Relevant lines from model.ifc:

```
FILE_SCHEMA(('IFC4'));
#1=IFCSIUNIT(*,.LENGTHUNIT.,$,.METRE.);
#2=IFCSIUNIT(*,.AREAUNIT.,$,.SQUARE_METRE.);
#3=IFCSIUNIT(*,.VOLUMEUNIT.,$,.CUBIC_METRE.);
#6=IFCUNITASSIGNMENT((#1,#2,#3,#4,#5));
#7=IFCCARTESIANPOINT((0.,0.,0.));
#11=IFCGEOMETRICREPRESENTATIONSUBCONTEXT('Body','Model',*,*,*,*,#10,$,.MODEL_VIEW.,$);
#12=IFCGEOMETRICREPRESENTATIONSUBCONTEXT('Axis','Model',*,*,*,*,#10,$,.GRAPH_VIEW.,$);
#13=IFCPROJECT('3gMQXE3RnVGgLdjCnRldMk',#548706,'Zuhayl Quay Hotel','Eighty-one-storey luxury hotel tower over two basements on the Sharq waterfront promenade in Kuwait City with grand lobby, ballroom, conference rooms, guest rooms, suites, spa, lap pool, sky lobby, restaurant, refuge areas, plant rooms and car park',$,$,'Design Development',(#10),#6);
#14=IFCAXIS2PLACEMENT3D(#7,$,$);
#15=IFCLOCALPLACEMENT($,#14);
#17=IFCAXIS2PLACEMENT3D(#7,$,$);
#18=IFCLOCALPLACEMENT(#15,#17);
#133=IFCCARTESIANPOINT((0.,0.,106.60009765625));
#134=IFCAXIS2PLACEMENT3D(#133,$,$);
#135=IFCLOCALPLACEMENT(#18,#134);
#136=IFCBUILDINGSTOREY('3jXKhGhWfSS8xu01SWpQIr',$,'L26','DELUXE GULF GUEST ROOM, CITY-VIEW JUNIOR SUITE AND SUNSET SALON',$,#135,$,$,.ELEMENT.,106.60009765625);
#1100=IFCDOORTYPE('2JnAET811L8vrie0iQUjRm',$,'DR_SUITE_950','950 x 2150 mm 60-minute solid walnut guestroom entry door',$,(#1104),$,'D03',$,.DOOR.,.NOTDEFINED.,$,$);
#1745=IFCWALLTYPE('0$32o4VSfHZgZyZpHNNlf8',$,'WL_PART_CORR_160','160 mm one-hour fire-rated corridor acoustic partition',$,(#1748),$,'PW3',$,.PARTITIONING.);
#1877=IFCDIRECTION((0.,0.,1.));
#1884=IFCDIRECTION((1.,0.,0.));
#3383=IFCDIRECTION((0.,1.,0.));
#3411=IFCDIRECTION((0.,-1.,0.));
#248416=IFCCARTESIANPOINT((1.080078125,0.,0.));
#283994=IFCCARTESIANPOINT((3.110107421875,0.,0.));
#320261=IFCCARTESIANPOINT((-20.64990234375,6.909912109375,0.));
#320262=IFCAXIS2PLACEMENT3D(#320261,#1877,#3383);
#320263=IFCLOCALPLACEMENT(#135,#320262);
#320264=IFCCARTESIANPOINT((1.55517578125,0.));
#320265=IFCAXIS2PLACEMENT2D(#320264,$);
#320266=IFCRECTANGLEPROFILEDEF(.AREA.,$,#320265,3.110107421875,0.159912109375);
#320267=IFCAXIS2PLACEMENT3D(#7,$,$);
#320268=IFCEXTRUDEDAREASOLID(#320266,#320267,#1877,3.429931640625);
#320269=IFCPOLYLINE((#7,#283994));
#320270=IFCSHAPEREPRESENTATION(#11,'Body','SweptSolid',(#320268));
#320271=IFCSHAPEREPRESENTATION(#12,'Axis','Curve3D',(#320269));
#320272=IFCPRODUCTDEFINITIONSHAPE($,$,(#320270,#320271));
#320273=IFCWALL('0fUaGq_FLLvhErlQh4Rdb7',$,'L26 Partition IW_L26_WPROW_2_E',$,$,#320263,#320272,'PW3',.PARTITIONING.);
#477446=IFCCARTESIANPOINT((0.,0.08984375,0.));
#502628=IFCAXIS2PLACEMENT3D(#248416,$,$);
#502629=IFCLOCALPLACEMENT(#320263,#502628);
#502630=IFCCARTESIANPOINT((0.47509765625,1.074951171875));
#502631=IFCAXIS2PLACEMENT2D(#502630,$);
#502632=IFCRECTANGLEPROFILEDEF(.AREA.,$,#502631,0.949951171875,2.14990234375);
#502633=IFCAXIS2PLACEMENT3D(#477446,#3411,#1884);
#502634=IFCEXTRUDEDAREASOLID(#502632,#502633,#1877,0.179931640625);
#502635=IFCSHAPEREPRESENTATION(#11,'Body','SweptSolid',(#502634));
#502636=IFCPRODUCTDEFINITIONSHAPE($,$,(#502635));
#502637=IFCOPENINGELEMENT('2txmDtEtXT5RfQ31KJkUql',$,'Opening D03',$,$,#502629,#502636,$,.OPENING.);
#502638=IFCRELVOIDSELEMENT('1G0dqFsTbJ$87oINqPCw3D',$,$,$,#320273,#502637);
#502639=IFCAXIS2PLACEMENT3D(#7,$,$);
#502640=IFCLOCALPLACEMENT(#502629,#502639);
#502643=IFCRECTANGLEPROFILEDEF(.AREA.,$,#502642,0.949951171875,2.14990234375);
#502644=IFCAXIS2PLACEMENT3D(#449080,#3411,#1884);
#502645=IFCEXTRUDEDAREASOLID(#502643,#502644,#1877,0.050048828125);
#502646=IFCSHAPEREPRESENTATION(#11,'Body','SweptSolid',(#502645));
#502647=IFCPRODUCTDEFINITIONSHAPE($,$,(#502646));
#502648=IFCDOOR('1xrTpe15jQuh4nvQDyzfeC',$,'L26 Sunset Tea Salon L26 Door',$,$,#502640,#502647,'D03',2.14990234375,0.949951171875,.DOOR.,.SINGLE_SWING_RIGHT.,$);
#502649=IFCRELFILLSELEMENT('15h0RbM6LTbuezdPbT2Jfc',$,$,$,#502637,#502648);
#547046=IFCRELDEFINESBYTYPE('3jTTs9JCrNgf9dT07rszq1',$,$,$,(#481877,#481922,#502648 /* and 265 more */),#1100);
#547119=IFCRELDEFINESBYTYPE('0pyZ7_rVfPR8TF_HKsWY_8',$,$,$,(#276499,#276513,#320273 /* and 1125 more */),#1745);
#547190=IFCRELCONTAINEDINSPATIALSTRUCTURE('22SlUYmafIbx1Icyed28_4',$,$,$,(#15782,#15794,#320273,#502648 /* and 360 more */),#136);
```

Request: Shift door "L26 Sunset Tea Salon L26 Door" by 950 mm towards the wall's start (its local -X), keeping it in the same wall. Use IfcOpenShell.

```python
import ifcopenshell
import ifcopenshell.api.geometry
import ifcopenshell.util.placement
import ifcopenshell.util.unit

model = ifcopenshell.open("model.ifc")
unit_scale = ifcopenshell.util.unit.calculate_unit_scale(model)

door = model.by_guid("1xrTpe15jQuh4nvQDyzfeC")
opening = door.FillsVoids[0].RelatingOpeningElement
wall = opening.VoidsElements[0].RelatingBuildingElement

wall_matrix = ifcopenshell.util.placement.get_local_placement(wall.ObjectPlacement)
shift = wall_matrix[:3, 0] * -0.95 / unit_scale
before = ifcopenshell.util.placement.get_local_placement(door.ObjectPlacement)[:3, 3].copy()

# The door is placed relative to its opening, so it follows when the opening moves.
matrix = ifcopenshell.util.placement.get_local_placement(opening.ObjectPlacement)
matrix[:3, 3] += shift
ifcopenshell.api.geometry.edit_object_placement(
    model, product=opening, matrix=matrix, is_si=False, should_transform_children=True
)

after = ifcopenshell.util.placement.get_local_placement(door.ObjectPlacement)[:3, 3]
print("door moved by", (after - before).round(3) + 0.0)

model.write("model_rev.ifc")
```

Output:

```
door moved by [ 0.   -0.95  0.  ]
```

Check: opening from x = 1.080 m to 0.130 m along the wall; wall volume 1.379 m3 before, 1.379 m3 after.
